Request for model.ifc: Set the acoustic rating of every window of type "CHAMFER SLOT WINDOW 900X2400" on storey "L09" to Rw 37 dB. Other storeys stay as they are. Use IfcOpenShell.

First a look at what the model holds.

```python
import ifcopenshell
import ifcopenshell.util.element

model = ifcopenshell.open("model.ifc")
print(model.schema)
storey = next(s for s in model.by_type("IfcBuildingStorey") if s.Name == "L09")
windows = [e for e in ifcopenshell.util.element.get_decomposition(storey) if e.is_a("IfcWindow")]
seen = {}
for e in windows:
    element_type = ifcopenshell.util.element.get_type(e)
    key = (element_type.Name if element_type != e and element_type else None, ifcopenshell.util.element.get_pset(e, "Pset_WindowCommon", "AcousticRating"))
    seen[key] = seen.get(key, 0) + 1
for (name, value), count in sorted(seen.items(), key=str):
    print(count, "x", name, "|", value)
```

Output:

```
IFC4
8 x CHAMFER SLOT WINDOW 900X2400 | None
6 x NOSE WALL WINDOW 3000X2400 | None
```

```python
import ifcopenshell
import ifcopenshell.api.pset
import ifcopenshell.util.element

model = ifcopenshell.open("model.ifc")

storey = next(s for s in model.by_type("IfcBuildingStorey") if s.Name == "L09")
windows = [e for e in ifcopenshell.util.element.get_decomposition(storey) if e.is_a("IfcWindow")]

count = 0
for e in windows:
    element_type = ifcopenshell.util.element.get_type(e)
    if element_type in (None, e) or element_type.Name != "CHAMFER SLOT WINDOW 900X2400":
        continue
    found = ifcopenshell.util.element.get_pset(e, "Pset_WindowCommon", should_inherit=False)
    if found:
        pset = model.by_id(found["id"])
        if len(ifcopenshell.util.element.get_elements_by_pset(pset)) > 1:
            pset = ifcopenshell.api.pset.unshare_pset(model, products=[e], pset=pset)[0]
    else:
        pset = ifcopenshell.api.pset.add_pset(model, product=e, name="Pset_WindowCommon")
    ifcopenshell.api.pset.edit_pset(model, pset=pset, properties={"AcousticRating": "Rw 37 dB"})
    count += 1

print(count, "windows updated")

model.write("model_v2.ifc")
```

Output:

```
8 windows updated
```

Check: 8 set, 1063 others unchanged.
